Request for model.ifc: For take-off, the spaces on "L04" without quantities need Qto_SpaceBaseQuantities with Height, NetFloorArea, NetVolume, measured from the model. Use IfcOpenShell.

First a look at what the model holds.

```python
import ifcopenshell
import ifcopenshell.util.element
import ifcopenshell.util.unit

model = ifcopenshell.open("model.ifc")
print(model.schema)
for unit_type in ("LENGTHUNIT", "AREAUNIT", "VOLUMEUNIT"):
    print(unit_type, ifcopenshell.util.unit.calculate_unit_scale(model, unit_type))
storey = next(s for s in model.by_type("IfcBuildingStorey") if s.Name == "L04")
spaces = [e for e in ifcopenshell.util.element.get_decomposition(storey) if e.is_a("IfcSpace")]
for e in sorted(spaces, key=lambda e: e.id()):
    print(e.id(), e.is_a(), e.Name, list(ifcopenshell.util.element.get_psets(e, qtos_only=True)), sep=" | ")
```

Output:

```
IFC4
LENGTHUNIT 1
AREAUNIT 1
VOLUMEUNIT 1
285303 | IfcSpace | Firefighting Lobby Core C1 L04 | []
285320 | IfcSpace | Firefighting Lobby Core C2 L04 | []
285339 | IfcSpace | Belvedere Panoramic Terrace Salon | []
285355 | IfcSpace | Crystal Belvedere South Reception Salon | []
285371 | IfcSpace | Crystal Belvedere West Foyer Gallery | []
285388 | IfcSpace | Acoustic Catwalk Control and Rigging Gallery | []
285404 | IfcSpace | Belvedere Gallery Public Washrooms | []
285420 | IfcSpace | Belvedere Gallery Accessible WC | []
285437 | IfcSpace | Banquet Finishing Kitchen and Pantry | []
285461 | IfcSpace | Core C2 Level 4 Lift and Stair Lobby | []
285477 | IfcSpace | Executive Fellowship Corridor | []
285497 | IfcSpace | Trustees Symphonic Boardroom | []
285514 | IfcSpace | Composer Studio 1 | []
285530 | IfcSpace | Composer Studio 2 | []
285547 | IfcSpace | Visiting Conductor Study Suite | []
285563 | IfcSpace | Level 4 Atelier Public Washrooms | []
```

```python
import ifcopenshell
import ifcopenshell.api.pset
import ifcopenshell.geom
import ifcopenshell.util.element
import ifcopenshell.util.shape
import ifcopenshell.util.unit

model = ifcopenshell.open("model.ifc")
unit_scale = ifcopenshell.util.unit.calculate_unit_scale(model)
area_scale = ifcopenshell.util.unit.calculate_unit_scale(model, "AREAUNIT")
volume_scale = ifcopenshell.util.unit.calculate_unit_scale(model, "VOLUMEUNIT")
settings = ifcopenshell.geom.settings()

storey = next(s for s in model.by_type("IfcBuildingStorey") if s.Name == "L04")
spaces = [e for e in ifcopenshell.util.element.get_decomposition(storey) if e.is_a("IfcSpace")]

for e in sorted(spaces, key=lambda e: e.id()):
    if ifcopenshell.util.element.get_psets(e, qtos_only=True, should_inherit=False):
        continue
    # Geometry comes back in metres, in the element's own axes.
    shape = ifcopenshell.geom.create_shape(settings, e)
    values = {
        "Height": ifcopenshell.util.shape.get_z(shape.geometry) / unit_scale,
        "NetFloorArea": ifcopenshell.util.shape.get_footprint_area(shape.geometry) / area_scale,
        "NetVolume": ifcopenshell.util.shape.get_volume(shape.geometry) / volume_scale,
    }
    qto = ifcopenshell.api.pset.add_qto(model, product=e, name="Qto_SpaceBaseQuantities")
    ifcopenshell.api.pset.edit_qto(model, qto=qto, properties=values)
    print(e.id(), {k: round(v, 3) for k, v in values.items()})

model.write("model_updated.ifc")
```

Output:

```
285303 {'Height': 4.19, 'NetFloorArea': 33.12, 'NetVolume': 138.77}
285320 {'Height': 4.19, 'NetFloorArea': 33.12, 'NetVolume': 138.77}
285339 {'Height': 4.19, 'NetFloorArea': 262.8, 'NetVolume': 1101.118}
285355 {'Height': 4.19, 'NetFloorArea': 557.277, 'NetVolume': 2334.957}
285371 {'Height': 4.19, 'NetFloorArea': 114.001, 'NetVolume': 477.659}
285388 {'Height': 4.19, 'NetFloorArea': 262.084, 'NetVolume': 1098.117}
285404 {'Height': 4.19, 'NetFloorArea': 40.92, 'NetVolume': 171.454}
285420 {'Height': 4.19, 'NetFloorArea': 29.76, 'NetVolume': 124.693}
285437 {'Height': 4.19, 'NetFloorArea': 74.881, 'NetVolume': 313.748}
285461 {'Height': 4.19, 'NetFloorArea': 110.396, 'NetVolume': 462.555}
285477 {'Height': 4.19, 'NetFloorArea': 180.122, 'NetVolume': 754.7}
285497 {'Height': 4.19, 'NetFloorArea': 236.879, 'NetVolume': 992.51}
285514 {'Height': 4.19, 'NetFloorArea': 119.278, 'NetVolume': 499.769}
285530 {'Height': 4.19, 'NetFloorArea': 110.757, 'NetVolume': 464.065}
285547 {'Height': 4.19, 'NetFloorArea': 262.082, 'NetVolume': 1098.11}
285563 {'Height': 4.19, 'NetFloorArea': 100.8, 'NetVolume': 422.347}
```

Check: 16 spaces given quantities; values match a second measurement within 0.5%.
